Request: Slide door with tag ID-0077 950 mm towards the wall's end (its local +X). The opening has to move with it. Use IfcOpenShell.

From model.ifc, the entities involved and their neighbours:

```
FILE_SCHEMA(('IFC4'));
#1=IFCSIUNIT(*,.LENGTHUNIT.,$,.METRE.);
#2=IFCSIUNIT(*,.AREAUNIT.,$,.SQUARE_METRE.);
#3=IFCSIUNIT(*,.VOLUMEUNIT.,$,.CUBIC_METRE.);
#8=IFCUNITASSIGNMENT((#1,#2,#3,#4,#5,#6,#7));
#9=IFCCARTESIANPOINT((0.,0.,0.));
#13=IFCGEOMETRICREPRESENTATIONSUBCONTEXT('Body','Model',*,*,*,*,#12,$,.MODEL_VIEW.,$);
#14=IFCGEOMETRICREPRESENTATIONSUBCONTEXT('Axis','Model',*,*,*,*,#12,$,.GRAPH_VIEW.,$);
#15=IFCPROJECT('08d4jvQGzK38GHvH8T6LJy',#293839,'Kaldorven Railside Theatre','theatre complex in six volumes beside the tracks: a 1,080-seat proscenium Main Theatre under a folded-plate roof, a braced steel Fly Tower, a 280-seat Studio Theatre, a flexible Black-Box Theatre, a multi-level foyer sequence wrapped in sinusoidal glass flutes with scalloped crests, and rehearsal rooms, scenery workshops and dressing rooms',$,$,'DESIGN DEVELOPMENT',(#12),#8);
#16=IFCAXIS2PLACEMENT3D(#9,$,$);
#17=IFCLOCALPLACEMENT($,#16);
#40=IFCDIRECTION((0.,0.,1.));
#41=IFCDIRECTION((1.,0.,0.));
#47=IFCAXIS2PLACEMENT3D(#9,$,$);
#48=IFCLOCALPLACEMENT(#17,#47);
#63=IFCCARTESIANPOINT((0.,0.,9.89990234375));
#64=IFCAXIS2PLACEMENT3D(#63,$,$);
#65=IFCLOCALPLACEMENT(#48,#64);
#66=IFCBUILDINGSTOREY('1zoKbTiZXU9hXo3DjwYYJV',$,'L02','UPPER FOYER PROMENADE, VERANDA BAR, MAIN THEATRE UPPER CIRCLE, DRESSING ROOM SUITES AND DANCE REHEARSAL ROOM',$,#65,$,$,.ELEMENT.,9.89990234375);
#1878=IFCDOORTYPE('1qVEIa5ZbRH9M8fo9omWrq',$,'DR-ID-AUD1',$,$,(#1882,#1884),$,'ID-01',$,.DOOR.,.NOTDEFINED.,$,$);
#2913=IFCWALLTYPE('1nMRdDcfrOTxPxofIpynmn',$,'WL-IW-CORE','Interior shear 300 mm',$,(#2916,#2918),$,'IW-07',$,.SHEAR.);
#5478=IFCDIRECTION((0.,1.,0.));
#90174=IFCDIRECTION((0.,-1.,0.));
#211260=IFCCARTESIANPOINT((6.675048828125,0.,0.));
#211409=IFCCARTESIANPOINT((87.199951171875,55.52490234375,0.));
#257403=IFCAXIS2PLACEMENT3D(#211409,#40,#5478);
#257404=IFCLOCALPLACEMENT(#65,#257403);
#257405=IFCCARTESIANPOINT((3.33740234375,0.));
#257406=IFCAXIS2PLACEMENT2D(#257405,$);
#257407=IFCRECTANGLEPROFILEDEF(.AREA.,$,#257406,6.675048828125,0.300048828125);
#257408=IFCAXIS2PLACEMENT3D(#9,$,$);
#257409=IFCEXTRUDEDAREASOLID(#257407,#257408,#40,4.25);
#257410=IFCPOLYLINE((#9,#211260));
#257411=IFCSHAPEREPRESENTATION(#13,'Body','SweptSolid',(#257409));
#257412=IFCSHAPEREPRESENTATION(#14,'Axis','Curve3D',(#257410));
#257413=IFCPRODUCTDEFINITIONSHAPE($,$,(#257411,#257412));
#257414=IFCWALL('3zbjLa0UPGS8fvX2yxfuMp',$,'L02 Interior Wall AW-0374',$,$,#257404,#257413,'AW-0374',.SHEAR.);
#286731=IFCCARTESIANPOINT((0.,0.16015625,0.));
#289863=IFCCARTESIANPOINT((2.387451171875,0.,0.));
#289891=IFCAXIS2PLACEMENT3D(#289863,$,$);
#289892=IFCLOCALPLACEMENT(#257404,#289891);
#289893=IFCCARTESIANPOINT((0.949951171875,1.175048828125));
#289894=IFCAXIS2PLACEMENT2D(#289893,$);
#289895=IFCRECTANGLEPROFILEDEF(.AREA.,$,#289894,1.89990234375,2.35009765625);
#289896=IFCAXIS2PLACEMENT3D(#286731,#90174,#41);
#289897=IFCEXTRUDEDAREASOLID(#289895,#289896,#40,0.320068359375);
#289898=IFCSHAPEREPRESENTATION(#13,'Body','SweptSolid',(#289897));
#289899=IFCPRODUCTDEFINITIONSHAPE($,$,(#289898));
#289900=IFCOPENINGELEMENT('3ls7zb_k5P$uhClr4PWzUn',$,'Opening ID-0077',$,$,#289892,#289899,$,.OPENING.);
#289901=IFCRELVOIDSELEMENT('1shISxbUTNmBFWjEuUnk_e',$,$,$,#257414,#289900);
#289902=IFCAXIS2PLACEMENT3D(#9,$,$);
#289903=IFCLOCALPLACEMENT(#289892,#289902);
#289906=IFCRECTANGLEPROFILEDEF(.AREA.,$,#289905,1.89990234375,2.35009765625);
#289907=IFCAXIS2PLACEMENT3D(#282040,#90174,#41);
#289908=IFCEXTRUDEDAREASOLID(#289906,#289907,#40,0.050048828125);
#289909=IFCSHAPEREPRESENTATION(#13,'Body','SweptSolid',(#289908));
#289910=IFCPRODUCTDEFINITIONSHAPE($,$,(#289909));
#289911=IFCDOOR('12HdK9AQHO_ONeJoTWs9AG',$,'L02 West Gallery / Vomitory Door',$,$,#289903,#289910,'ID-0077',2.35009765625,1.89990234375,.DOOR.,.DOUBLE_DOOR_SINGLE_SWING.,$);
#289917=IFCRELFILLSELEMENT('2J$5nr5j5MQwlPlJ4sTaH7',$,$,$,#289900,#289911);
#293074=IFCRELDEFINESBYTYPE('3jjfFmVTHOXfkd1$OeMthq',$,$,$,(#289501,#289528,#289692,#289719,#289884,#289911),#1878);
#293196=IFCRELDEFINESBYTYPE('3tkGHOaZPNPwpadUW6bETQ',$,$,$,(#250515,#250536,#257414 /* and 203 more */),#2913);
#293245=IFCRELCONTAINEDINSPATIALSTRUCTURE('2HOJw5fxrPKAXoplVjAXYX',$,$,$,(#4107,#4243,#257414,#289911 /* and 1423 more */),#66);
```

```python
import ifcopenshell
import ifcopenshell.api.geometry
import ifcopenshell.util.placement

model = ifcopenshell.open("model.ifc")

door = model.by_id(289911)
opening = door.FillsVoids[0].RelatingOpeningElement
wall = opening.VoidsElements[0].RelatingBuildingElement

wall_matrix = ifcopenshell.util.placement.get_local_placement(wall.ObjectPlacement)
shift = wall_matrix[:3, 0] * 0.95
before = ifcopenshell.util.placement.get_local_placement(door.ObjectPlacement)[:3, 3].copy()

# The door is placed relative to its opening, so it follows when the opening moves.
matrix = ifcopenshell.util.placement.get_local_placement(opening.ObjectPlacement)
matrix[:3, 3] += shift
ifcopenshell.api.geometry.edit_object_placement(
    model, product=opening, matrix=matrix, is_si=False, should_transform_children=True
)

after = ifcopenshell.util.placement.get_local_placement(door.ObjectPlacement)[:3, 3]
print("door moved by", (after - before).round(3) + 0.0)

model.write("model_updated.ifc")
```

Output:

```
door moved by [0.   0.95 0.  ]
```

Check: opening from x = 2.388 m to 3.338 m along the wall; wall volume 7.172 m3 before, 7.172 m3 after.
